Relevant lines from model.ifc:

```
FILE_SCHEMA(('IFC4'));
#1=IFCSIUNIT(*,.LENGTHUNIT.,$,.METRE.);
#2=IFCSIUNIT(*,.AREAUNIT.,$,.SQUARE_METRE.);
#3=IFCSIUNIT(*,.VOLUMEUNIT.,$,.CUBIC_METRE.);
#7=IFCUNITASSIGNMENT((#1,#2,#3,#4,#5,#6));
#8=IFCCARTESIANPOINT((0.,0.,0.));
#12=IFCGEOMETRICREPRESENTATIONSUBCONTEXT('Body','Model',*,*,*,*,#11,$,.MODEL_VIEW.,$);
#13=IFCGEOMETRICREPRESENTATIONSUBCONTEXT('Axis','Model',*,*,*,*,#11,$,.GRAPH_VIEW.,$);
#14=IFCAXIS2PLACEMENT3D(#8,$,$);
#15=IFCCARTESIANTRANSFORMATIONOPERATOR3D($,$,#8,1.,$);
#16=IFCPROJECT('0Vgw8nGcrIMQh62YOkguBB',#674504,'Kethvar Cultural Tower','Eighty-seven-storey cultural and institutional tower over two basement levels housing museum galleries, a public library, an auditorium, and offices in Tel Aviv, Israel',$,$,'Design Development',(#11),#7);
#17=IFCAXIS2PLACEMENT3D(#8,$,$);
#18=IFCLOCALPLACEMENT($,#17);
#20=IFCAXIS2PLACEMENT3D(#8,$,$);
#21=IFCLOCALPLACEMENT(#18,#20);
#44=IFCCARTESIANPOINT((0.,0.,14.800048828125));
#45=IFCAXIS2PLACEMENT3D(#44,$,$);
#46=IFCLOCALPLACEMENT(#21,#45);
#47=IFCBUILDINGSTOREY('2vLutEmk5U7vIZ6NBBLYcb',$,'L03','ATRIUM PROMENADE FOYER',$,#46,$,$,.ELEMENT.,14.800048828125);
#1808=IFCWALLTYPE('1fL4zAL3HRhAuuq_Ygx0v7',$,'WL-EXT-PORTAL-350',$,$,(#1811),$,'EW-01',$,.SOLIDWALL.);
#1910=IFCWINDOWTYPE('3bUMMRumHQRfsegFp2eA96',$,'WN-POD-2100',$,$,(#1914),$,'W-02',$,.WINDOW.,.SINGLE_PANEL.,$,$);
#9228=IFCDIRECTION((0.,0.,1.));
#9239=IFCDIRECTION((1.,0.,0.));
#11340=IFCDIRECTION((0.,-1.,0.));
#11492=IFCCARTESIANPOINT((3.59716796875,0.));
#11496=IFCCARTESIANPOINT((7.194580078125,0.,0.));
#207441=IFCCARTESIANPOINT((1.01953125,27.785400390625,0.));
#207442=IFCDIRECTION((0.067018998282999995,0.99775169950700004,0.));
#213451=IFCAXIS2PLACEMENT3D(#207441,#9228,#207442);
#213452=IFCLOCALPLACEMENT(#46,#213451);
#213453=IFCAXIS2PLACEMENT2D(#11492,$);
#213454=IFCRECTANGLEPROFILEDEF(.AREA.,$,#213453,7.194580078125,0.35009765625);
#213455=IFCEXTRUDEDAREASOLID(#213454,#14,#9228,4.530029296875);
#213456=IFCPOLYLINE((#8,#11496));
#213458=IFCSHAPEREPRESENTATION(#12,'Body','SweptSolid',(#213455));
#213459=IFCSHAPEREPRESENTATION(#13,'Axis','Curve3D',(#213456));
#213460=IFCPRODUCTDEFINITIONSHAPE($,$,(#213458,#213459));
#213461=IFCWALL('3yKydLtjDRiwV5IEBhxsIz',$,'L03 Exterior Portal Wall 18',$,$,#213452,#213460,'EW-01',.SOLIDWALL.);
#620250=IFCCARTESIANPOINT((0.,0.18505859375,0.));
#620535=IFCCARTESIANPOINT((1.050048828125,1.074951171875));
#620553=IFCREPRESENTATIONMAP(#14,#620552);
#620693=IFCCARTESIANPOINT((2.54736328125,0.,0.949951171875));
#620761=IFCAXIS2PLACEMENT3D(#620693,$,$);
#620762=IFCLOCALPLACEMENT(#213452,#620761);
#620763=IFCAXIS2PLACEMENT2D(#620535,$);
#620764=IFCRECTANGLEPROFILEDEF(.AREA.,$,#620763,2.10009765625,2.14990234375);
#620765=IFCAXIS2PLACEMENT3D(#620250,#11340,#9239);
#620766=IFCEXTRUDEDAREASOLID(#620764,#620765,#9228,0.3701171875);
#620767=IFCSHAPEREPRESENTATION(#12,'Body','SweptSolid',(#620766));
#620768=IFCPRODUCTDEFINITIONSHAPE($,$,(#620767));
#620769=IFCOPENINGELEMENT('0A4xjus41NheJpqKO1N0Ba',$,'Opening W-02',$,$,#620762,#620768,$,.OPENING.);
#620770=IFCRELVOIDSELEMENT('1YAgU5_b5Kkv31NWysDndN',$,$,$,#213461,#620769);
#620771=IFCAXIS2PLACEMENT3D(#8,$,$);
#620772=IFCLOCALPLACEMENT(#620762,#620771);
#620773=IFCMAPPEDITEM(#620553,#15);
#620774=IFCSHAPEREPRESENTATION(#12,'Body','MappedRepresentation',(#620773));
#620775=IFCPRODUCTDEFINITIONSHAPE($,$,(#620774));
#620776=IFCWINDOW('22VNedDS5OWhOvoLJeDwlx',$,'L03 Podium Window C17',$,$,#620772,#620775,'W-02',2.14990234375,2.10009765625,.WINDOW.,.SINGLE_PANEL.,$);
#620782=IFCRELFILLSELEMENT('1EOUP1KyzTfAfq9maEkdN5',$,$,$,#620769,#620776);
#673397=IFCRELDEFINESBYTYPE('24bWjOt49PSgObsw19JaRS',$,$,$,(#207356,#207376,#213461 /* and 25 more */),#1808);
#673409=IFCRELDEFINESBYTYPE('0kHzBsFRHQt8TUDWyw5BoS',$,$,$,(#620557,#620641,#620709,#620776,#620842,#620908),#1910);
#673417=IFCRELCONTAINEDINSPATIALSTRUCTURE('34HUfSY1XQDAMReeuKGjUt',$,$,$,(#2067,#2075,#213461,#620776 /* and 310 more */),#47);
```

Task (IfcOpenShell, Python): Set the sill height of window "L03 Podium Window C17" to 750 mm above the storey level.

```python
import numpy as np
import ifcopenshell
import ifcopenshell.api.geometry
import ifcopenshell.geom
import ifcopenshell.util.element
import ifcopenshell.util.placement
import ifcopenshell.util.shape
import ifcopenshell.util.unit

model = ifcopenshell.open("model.ifc")
unit_scale = ifcopenshell.util.unit.calculate_unit_scale(model)

window = model.by_guid("22VNedDS5OWhOvoLJeDwlx")
opening = window.FillsVoids[0].RelatingOpeningElement
storey = ifcopenshell.util.element.get_container(window, ifc_class="IfcBuildingStorey")
level = ifcopenshell.util.placement.get_local_placement(storey.ObjectPlacement)[2, 3]

# The opening's origin need not be at the sill, so measure its lowest point.
shape = ifcopenshell.geom.create_shape(ifcopenshell.geom.settings(), opening)
bottom = ifcopenshell.util.shape.get_shape_bottom_elevation(shape, shape.geometry) / unit_scale
dz = level + 0.75 / unit_scale - bottom

shift = np.array([0.0, 0.0, dz])
# The window is placed relative to its opening, so it follows when the opening moves.
matrix = ifcopenshell.util.placement.get_local_placement(opening.ObjectPlacement)
matrix[:3, 3] += shift
ifcopenshell.api.geometry.edit_object_placement(
    model, product=opening, matrix=matrix, is_si=False, should_transform_children=True
)

print(f"moved by {dz * unit_scale:+.3f} m")

model.write("model_edited.ifc")
```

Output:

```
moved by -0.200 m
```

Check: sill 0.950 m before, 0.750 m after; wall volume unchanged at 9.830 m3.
